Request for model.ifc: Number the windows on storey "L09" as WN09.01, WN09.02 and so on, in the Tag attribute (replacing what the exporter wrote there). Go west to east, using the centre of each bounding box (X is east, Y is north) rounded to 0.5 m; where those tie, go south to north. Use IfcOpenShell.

First a look at what the model holds.

```python
import ifcopenshell
import ifcopenshell.util.element
import ifcopenshell.util.placement

model = ifcopenshell.open("model.ifc")
print(model.schema)
storey = next(s for s in model.by_type("IfcBuildingStorey") if s.Name == "L09")
windows = [e for e in ifcopenshell.util.element.get_decomposition(storey) if e.is_a("IfcWindow")]
for e in sorted(windows, key=lambda e: e.id()):
    origin = ifcopenshell.util.placement.get_local_placement(e.ObjectPlacement)[:3, 3]
    print(e.id(), e.Tag, e.Name, origin.round(2) + 0.0, sep=" | ")
```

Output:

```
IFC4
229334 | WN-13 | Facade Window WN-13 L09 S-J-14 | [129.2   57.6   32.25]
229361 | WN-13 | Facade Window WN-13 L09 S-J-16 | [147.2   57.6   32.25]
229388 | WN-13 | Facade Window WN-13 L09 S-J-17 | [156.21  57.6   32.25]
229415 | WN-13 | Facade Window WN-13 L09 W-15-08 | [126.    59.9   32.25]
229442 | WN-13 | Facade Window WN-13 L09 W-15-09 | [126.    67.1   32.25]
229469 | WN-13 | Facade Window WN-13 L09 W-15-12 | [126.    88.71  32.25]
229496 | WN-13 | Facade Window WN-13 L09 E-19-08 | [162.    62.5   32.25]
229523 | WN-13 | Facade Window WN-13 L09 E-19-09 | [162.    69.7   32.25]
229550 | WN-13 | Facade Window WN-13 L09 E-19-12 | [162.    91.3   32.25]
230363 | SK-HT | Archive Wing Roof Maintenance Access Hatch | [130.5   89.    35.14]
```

```python
import ifcopenshell
import ifcopenshell.geom
import ifcopenshell.util.element
import ifcopenshell.util.shape

model = ifcopenshell.open("model.ifc")
settings = ifcopenshell.geom.settings()
settings.set("use-world-coords", True)


def centre(element):
    shape = ifcopenshell.geom.create_shape(settings, element)
    return ifcopenshell.util.shape.get_bbox_centroid(shape.geometry)


storey = next(s for s in model.by_type("IfcBuildingStorey") if s.Name == "L09")
windows = [e for e in ifcopenshell.util.element.get_decomposition(storey) if e.is_a("IfcWindow")]

# Insertion points can sit at a corner or the storey origin, so sort by the geometry (in metres).
centres = {e: centre(e) for e in windows}
windows.sort(key=lambda e: (round(centres[e][0] / 0.5), centres[e][1]))

for i, e in enumerate(windows, start=1):
    number = f"WN09.{i:02d}"
    e.Tag = number
    print(e.id(), number)

model.write("model_v2.ifc")
```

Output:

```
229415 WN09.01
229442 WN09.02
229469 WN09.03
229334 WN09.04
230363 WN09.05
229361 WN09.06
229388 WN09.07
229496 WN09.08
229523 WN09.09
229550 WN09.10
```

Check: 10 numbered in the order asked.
